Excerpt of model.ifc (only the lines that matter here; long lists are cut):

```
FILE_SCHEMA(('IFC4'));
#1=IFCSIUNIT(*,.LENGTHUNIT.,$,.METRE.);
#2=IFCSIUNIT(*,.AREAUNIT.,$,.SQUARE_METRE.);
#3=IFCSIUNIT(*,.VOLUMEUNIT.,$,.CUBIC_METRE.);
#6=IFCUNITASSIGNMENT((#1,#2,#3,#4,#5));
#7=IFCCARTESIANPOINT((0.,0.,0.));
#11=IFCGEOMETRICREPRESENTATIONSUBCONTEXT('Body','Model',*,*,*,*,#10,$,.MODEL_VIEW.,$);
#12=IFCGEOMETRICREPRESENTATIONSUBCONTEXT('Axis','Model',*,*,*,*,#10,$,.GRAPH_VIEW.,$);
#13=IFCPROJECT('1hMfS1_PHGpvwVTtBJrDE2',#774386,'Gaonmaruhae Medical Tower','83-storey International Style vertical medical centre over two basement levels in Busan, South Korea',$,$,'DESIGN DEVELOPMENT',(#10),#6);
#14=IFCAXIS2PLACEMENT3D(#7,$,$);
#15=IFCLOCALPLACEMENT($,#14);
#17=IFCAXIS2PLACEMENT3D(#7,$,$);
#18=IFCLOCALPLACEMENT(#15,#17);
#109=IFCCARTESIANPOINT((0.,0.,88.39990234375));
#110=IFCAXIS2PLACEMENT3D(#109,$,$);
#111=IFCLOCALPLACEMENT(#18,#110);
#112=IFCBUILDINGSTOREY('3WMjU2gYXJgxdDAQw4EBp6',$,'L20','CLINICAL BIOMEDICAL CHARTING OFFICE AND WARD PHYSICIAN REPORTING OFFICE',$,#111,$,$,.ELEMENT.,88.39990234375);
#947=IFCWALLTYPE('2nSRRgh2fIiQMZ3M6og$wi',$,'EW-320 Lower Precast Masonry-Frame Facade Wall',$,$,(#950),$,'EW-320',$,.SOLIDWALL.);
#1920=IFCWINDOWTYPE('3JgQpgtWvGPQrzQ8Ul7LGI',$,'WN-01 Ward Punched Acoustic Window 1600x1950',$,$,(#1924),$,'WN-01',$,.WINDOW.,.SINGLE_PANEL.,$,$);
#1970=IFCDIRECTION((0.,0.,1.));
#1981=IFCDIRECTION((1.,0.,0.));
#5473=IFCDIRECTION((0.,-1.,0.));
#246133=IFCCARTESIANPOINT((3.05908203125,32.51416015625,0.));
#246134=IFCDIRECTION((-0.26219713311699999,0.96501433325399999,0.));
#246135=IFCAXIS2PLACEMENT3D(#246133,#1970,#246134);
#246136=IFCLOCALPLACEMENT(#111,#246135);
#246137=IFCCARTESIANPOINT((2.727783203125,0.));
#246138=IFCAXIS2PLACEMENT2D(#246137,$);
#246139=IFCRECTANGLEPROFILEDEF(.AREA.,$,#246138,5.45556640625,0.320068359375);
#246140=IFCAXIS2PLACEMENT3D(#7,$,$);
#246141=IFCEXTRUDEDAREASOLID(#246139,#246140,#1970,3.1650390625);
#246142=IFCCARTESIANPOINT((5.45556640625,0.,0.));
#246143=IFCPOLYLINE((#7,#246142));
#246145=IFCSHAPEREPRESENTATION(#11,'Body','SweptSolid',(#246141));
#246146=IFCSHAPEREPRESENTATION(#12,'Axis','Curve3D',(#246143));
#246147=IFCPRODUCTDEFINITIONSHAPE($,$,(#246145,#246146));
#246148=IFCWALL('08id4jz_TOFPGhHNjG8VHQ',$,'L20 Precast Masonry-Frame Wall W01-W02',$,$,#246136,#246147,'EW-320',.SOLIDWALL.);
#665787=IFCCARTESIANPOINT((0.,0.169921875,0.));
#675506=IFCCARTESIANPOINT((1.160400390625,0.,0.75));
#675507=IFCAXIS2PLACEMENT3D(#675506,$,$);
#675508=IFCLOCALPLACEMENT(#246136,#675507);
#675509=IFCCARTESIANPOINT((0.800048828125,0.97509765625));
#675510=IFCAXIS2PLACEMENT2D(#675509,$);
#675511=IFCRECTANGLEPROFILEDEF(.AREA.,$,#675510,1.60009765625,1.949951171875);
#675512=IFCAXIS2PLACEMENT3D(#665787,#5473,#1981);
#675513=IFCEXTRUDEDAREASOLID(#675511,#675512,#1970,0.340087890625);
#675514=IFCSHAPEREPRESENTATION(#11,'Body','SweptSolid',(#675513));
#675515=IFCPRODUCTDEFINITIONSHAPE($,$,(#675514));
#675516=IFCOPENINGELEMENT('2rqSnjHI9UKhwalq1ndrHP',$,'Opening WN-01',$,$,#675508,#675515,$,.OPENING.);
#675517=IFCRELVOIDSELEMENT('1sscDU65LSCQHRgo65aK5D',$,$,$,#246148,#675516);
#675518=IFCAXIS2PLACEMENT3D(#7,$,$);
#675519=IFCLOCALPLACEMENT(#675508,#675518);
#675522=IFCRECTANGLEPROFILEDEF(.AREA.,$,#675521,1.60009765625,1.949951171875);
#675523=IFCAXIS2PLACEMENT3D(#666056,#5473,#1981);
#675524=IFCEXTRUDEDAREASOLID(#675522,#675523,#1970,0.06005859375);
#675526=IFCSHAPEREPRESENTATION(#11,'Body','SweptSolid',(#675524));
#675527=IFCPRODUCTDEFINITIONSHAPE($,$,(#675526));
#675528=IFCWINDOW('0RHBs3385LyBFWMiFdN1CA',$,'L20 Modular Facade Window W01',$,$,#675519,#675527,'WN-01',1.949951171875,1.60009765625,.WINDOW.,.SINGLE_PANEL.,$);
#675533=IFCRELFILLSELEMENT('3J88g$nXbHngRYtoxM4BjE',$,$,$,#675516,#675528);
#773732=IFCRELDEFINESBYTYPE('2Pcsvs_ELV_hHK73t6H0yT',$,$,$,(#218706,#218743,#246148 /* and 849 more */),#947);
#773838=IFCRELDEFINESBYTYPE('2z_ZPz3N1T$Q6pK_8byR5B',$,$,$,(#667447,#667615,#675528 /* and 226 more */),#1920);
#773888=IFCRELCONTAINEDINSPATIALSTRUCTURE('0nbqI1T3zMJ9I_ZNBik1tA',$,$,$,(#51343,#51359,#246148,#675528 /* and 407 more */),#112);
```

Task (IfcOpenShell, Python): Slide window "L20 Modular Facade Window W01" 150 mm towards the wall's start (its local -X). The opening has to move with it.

```python
import ifcopenshell
import ifcopenshell.api.geometry
import ifcopenshell.util.placement
import ifcopenshell.util.unit

model = ifcopenshell.open("model.ifc")
unit_scale = ifcopenshell.util.unit.calculate_unit_scale(model)

window = model.by_guid("0RHBs3385LyBFWMiFdN1CA")
opening = window.FillsVoids[0].RelatingOpeningElement
wall = opening.VoidsElements[0].RelatingBuildingElement

wall_matrix = ifcopenshell.util.placement.get_local_placement(wall.ObjectPlacement)
shift = wall_matrix[:3, 0] * -0.15 / unit_scale
before = ifcopenshell.util.placement.get_local_placement(window.ObjectPlacement)[:3, 3].copy()

# The window is placed relative to its opening, so it follows when the opening moves.
matrix = ifcopenshell.util.placement.get_local_placement(opening.ObjectPlacement)
matrix[:3, 3] += shift
ifcopenshell.api.geometry.edit_object_placement(
    model, product=opening, matrix=matrix, is_si=False, should_transform_children=True
)

after = ifcopenshell.util.placement.get_local_placement(window.ObjectPlacement)[:3, 3]
print("window moved by", (after - before).round(3) + 0.0)

model.write("model_updated.ifc")
```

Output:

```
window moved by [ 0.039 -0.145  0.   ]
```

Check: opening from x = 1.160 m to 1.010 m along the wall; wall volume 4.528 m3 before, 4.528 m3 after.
